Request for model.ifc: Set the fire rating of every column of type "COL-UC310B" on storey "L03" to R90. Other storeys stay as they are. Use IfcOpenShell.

First a look at what the model holds.

```python
import ifcopenshell
import ifcopenshell.util.element

model = ifcopenshell.open("model.ifc")
print(model.schema)
storey = next(s for s in model.by_type("IfcBuildingStorey") if s.Name == "L03")
columns = [e for e in ifcopenshell.util.element.get_decomposition(storey) if e.is_a("IfcColumn")]
seen = {}
for e in columns:
    element_type = ifcopenshell.util.element.get_type(e)
    key = (element_type.Name if element_type != e and element_type else None, ifcopenshell.util.element.get_pset(e, "Pset_ColumnCommon", "FireRating"))
    seen[key] = seen.get(key, 0) + 1
for (name, value), count in sorted(seen.items(), key=str):
    print(count, "x", name, "|", value)
```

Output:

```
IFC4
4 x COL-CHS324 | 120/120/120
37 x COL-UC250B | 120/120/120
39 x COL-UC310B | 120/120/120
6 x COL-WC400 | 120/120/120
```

```python
import ifcopenshell
import ifcopenshell.api.pset
import ifcopenshell.util.element

model = ifcopenshell.open("model.ifc")

storey = next(s for s in model.by_type("IfcBuildingStorey") if s.Name == "L03")
columns = [e for e in ifcopenshell.util.element.get_decomposition(storey) if e.is_a("IfcColumn")]

count = 0
for e in columns:
    element_type = ifcopenshell.util.element.get_type(e)
    if element_type in (None, e) or element_type.Name != "COL-UC310B":
        continue
    # add_pset returns the element's existing set when there is one.
    pset = ifcopenshell.api.pset.add_pset(model, product=e, name="Pset_ColumnCommon")
    ifcopenshell.api.pset.edit_pset(model, pset=pset, properties={"FireRating": "R90"})
    count += 1

print(count, "columns updated")

model.write("model-out.ifc")
```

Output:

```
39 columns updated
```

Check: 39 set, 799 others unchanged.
